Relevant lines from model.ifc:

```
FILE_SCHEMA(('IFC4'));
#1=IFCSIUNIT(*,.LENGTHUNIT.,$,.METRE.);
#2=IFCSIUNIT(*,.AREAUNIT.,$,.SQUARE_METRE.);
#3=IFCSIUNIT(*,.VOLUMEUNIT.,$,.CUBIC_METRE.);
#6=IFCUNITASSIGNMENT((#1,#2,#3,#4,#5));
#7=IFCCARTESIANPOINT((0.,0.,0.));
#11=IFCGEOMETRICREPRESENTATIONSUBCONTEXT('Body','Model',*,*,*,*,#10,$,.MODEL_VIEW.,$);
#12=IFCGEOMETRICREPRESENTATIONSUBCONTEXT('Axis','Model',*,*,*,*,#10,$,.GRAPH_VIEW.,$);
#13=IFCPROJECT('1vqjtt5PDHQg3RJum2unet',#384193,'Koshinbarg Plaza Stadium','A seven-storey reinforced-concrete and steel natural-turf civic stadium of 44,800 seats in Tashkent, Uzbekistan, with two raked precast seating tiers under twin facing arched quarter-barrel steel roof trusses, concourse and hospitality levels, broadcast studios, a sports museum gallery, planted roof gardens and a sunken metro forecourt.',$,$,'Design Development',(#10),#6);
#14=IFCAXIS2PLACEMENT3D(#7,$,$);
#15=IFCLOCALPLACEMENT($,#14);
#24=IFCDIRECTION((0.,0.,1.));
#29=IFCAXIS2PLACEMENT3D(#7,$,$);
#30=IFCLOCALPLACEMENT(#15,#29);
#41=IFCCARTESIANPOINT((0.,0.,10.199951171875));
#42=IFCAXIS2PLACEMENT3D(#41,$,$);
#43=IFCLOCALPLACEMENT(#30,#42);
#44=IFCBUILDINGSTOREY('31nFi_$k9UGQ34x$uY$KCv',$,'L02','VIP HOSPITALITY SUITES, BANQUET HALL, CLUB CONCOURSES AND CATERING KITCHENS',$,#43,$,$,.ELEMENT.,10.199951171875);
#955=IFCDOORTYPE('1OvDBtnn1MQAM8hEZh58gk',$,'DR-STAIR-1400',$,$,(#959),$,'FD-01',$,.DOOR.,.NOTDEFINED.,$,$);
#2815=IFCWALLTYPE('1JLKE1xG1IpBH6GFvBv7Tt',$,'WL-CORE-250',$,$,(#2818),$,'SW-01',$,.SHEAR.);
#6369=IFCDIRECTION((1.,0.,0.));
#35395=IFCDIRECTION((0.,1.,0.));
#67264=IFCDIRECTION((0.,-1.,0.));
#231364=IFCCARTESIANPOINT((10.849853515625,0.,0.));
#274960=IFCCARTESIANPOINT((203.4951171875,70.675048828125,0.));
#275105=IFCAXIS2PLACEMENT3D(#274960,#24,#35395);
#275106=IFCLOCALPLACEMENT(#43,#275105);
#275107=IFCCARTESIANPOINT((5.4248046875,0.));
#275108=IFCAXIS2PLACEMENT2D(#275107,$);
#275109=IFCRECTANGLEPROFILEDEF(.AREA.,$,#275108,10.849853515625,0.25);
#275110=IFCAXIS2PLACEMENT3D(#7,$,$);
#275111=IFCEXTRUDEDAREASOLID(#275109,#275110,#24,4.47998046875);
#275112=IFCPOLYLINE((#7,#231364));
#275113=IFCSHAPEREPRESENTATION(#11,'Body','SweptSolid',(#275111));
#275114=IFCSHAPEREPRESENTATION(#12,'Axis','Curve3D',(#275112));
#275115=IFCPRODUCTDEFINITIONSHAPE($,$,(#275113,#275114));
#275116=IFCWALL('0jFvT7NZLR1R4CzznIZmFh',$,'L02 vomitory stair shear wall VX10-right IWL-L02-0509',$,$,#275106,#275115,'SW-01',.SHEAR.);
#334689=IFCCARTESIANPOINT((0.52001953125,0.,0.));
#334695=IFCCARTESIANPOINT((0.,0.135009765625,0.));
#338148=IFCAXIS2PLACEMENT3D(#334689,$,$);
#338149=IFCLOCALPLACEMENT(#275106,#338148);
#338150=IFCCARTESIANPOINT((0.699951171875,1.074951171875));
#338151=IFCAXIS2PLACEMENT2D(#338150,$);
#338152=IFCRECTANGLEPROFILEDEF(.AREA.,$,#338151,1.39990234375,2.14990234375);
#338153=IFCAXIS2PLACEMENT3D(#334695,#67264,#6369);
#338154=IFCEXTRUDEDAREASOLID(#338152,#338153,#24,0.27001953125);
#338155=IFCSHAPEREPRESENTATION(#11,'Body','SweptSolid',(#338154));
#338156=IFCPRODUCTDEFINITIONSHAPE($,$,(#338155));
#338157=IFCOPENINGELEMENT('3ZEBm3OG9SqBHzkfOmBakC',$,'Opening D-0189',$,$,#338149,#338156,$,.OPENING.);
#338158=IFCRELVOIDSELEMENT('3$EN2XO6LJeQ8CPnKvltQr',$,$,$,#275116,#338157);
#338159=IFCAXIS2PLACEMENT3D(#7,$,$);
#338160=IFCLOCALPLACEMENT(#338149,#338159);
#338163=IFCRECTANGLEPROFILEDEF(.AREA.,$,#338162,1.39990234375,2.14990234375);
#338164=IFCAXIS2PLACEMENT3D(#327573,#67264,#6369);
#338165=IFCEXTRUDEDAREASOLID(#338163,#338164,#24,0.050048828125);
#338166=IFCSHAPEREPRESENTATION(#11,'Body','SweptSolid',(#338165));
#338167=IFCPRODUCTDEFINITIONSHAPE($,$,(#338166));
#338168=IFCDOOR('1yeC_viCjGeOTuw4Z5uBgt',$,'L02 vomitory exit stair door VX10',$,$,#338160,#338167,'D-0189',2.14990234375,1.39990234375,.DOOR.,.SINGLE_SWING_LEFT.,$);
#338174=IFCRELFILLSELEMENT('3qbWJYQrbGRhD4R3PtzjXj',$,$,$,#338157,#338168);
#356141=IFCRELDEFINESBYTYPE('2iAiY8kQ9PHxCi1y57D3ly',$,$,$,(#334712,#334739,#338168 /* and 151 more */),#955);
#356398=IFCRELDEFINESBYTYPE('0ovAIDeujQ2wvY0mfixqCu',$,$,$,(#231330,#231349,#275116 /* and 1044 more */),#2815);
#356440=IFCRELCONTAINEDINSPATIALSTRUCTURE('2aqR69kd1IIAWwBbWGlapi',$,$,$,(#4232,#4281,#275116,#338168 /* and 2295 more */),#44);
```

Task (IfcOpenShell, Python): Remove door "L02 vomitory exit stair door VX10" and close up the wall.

```python
import ifcopenshell
import ifcopenshell.api.feature
import ifcopenshell.api.root
import ifcopenshell.geom
import ifcopenshell.util.shape

model = ifcopenshell.open("model.ifc")
settings = ifcopenshell.geom.settings()


def volume(element):
    """Net volume in cubic metres, openings subtracted."""
    shape = ifcopenshell.geom.create_shape(settings, element)
    return ifcopenshell.util.shape.get_volume(shape.geometry)


door = model.by_id(338168)
opening = door.FillsVoids[0].RelatingOpeningElement
wall = opening.VoidsElements[0].RelatingBuildingElement
before = volume(wall)

ifcopenshell.api.root.remove_product(model, product=door)
ifcopenshell.api.feature.remove_feature(model, feature=opening)

after = volume(wall)

print(f"wall volume {before:.3f} -> {after:.3f} m3")

model.write("model_edited.ifc")
```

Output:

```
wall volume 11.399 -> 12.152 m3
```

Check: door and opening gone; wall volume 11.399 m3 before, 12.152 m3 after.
